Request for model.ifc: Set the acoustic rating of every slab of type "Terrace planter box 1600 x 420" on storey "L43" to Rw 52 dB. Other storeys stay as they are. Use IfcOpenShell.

First a look at what the model holds.

```python
import ifcopenshell
import ifcopenshell.util.element

model = ifcopenshell.open("model.ifc")
print(model.schema)
storey = next(s for s in model.by_type("IfcBuildingStorey") if s.Name == "L43")
slabs = [e for e in ifcopenshell.util.element.get_decomposition(storey) if e.is_a("IfcSlab")]
seen = {}
for e in slabs:
    element_type = ifcopenshell.util.element.get_type(e)
    key = (element_type.Name if element_type != e and element_type else None, ifcopenshell.util.element.get_pset(e, "Pset_SlabCommon", "AcousticRating"))
    seen[key] = seen.get(key, 0) + 1
for (name, value), count in sorted(seen.items(), key=str):
    print(count, "x", name, "|", value)
```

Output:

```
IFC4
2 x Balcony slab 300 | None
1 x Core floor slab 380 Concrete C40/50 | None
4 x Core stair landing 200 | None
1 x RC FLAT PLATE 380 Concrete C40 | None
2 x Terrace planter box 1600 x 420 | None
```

```python
import ifcopenshell
import ifcopenshell.api.pset
import ifcopenshell.util.element

model = ifcopenshell.open("model.ifc")

storey = next(s for s in model.by_type("IfcBuildingStorey") if s.Name == "L43")
slabs = [e for e in ifcopenshell.util.element.get_decomposition(storey) if e.is_a("IfcSlab")]

count = 0
for e in slabs:
    element_type = ifcopenshell.util.element.get_type(e)
    if element_type in (None, e) or element_type.Name != "Terrace planter box 1600 x 420":
        continue
    # add_pset returns the element's existing set when there is one.
    pset = ifcopenshell.api.pset.add_pset(model, product=e, name="Pset_SlabCommon")
    ifcopenshell.api.pset.edit_pset(model, pset=pset, properties={"AcousticRating": "Rw 52 dB"})
    count += 1

print(count, "slabs updated")

model.write("model-out.ifc")
```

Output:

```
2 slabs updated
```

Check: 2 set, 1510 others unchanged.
